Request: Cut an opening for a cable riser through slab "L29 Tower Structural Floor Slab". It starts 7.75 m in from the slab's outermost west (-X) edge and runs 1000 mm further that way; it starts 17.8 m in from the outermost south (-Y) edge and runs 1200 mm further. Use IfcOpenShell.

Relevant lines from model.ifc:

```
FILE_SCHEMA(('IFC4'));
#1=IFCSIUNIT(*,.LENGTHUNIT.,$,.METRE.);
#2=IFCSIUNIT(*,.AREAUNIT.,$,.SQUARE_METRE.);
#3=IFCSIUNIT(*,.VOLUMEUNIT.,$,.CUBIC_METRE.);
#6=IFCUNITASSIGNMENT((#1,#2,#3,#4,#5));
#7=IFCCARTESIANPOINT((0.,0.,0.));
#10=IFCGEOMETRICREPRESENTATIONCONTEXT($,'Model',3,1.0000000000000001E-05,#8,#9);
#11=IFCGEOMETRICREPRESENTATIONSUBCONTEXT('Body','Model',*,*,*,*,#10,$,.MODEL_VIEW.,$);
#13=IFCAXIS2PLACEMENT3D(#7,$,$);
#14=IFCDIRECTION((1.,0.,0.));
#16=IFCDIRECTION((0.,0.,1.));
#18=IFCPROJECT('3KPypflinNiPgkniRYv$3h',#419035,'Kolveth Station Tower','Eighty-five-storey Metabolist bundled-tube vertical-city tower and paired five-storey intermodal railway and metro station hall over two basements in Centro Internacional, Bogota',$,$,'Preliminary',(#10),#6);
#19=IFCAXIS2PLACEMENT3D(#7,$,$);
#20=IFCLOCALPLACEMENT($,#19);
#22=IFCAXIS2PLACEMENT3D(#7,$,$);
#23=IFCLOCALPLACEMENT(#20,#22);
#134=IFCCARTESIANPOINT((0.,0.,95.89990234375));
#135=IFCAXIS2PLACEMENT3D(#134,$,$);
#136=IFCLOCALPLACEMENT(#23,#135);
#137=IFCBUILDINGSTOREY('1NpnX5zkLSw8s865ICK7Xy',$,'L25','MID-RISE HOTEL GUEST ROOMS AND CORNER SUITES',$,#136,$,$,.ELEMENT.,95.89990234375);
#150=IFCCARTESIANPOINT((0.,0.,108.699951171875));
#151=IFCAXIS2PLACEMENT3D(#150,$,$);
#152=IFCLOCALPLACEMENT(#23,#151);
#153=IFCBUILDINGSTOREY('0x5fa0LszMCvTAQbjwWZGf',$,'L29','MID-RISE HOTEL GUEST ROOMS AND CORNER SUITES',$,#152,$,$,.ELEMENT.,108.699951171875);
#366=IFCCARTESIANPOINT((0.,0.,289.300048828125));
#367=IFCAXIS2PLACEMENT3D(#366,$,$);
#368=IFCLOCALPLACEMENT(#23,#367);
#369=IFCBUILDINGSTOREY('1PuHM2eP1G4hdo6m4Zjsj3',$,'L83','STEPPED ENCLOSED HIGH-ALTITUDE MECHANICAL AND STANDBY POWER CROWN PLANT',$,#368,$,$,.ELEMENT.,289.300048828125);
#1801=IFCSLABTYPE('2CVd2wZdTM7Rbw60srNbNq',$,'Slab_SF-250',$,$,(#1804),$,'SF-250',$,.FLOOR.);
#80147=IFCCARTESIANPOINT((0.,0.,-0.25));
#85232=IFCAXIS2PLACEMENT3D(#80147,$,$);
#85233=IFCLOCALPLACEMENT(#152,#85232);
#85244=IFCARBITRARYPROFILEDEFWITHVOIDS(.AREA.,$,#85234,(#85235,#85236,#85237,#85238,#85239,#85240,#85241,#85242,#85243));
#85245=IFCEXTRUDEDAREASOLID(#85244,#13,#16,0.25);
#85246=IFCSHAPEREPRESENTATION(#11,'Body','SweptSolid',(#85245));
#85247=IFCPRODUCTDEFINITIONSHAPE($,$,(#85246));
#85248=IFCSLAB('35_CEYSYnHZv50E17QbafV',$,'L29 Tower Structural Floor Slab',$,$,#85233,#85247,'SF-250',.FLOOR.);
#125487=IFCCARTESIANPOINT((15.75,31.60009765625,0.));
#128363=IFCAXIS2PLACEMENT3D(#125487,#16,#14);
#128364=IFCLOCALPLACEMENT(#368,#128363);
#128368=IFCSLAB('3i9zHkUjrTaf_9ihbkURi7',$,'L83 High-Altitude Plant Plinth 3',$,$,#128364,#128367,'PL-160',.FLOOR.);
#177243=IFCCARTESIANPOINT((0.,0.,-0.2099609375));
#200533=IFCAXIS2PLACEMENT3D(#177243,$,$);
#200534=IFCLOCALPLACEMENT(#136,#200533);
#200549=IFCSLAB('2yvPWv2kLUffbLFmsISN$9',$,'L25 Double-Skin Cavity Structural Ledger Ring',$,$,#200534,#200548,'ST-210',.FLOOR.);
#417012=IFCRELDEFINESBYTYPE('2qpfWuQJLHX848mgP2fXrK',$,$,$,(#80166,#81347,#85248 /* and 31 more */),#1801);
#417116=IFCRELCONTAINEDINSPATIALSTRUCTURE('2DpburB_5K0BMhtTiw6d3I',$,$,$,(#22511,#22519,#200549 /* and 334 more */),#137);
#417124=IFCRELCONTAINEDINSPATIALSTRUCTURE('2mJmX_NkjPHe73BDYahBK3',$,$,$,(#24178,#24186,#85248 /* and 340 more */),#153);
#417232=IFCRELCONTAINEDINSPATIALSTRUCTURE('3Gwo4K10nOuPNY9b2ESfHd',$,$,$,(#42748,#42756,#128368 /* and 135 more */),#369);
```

```python
import numpy as np
import ifcopenshell
import ifcopenshell.api.feature
import ifcopenshell.api.geometry
import ifcopenshell.api.root
import ifcopenshell.geom
import ifcopenshell.util.placement
import ifcopenshell.util.representation
import ifcopenshell.util.shape
import ifcopenshell.util.unit

model = ifcopenshell.open("model.ifc")
unit_scale = ifcopenshell.util.unit.calculate_unit_scale(model)
settings = ifcopenshell.geom.settings()


def volume(element):
    """Net volume in cubic metres, openings subtracted."""
    shape = ifcopenshell.geom.create_shape(settings, element)
    return ifcopenshell.util.shape.get_volume(shape.geometry)


slab = model.by_guid("35_CEYSYnHZv50E17QbafV")
before = volume(slab)

# Extent in the slab's own axes, in metres. The edges named are its -X and -Y sides.
slab_shape = ifcopenshell.geom.create_shape(settings, slab)
vertices = ifcopenshell.util.shape.get_vertices(slab_shape.geometry)
x_min, y_min, bottom = vertices.min(axis=0)
top = vertices[:, 2].max()

opening = ifcopenshell.api.root.create_entity(model, ifc_class="IfcOpeningElement", name="Cable riser opening", predefined_type="OPENING")
context = ifcopenshell.util.representation.get_context(model, "Model", "Body", "MODEL_VIEW")
width, depth = 1, 1.2
outline = [(0.0, 0.0), (width, 0.0), (width, depth), (0.0, depth), (0.0, 0.0)]
# Overshoot both faces by 50 mm so the cut is clean.
shape = ifcopenshell.api.geometry.add_slab_representation(
    model, context=context, depth=top - bottom + 0.1, polyline=outline
)
ifcopenshell.api.geometry.assign_representation(model, product=opening, representation=shape)

matrix = ifcopenshell.util.placement.get_local_placement(slab.ObjectPlacement)
matrix[:, 3] = matrix @ np.append(np.array([x_min + 7.75, y_min + 17.8, bottom - 0.05]) / unit_scale, 1.0)
ifcopenshell.api.geometry.edit_object_placement(model, product=opening, matrix=matrix, is_si=False)
ifcopenshell.api.feature.add_feature(model, feature=opening, element=slab)

after = volume(slab)

print(f"slab volume {before:.3f} -> {after:.3f} m3")

model.write("model_edited.ifc")
```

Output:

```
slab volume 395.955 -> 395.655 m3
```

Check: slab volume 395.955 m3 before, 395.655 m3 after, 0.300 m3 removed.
